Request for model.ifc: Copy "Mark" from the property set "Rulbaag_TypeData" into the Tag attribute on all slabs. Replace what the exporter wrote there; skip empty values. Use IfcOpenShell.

First a look at what the model holds.

```python
import ifcopenshell
import ifcopenshell.util.element

model = ifcopenshell.open("model.ifc")
print(model.schema)
slabs = model.by_type("IfcSlab")
print(len(slabs), "slabs")
for e in slabs[:8]:
    source = ifcopenshell.util.element.get_pset(e, "Rulbaag_TypeData", "Mark")
    target = e.Tag
    print(e.id(), repr(source), repr(target), sep=" | ")
```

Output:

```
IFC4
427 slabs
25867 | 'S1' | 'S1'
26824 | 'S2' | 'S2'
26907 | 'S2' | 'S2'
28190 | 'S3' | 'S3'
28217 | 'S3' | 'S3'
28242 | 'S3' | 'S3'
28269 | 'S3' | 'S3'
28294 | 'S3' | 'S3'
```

```python
import ifcopenshell
import ifcopenshell.util.element

model = ifcopenshell.open("model.ifc")

count = 0
for e in model.by_type("IfcSlab"):
    value = ifcopenshell.util.element.get_pset(e, "Rulbaag_TypeData", "Mark")
    current = e.Tag
    if not value or not value.strip() or current == value:
        continue
    e.Tag = value
    count += 1

print(count, "slabs updated")

model.write("model_v2.ifc")
```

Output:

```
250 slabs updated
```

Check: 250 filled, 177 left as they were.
